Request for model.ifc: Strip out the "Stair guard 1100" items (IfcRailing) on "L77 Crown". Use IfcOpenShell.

First a look at what the model holds.

```python
import ifcopenshell
import ifcopenshell.util.element

model = ifcopenshell.open("model.ifc")
print(model.schema)
storey = next(s for s in model.by_type("IfcBuildingStorey") if s.Name == "L77 Crown")
railings = [e for e in ifcopenshell.util.element.get_decomposition(storey) if e.is_a("IfcRailing")]
seen = {}
for e in railings:
    element_type = ifcopenshell.util.element.get_type(e)
    name = element_type.Name if element_type not in (None, e) else None
    seen[name] = seen.get(name, 0) + 1
for name, count in sorted(seen.items(), key=str):
    print(count, "x", name)
```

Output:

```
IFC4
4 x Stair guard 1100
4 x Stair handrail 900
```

```python
import ifcopenshell
import ifcopenshell.api.root
import ifcopenshell.util.element

model = ifcopenshell.open("model.ifc")

storey = next(s for s in model.by_type("IfcBuildingStorey") if s.Name == "L77 Crown")
railings = [e for e in ifcopenshell.util.element.get_decomposition(storey) if e.is_a("IfcRailing")]
targets = [e for e in railings if (t := ifcopenshell.util.element.get_type(e)) not in (None, e) and t.Name == "Stair guard 1100"]

for e in targets:
    ifcopenshell.api.root.remove_product(model, product=e)
print(len(targets), "removed")

model.write("model_v2.ifc")
```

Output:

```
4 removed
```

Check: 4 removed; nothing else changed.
